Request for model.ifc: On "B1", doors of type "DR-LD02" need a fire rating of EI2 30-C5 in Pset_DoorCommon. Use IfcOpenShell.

First a look at what the model holds.

```python
import ifcopenshell
import ifcopenshell.util.element

model = ifcopenshell.open("model.ifc")
print(model.schema)
storey = next(s for s in model.by_type("IfcBuildingStorey") if s.Name == "B1")
doors = [e for e in ifcopenshell.util.element.get_decomposition(storey) if e.is_a("IfcDoor")]
seen = {}
for e in doors:
    element_type = ifcopenshell.util.element.get_type(e)
    key = (element_type.Name if element_type != e and element_type else None, ifcopenshell.util.element.get_pset(e, "Pset_DoorCommon", "FireRating"))
    seen[key] = seen.get(key, 0) + 1
for (name, value), count in sorted(seen.items(), key=str):
    print(count, "x", name, "|", value)
```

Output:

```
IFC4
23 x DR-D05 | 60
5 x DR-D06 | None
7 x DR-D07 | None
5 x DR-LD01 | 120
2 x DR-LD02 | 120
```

```python
import ifcopenshell
import ifcopenshell.api.pset
import ifcopenshell.util.element

model = ifcopenshell.open("model.ifc")

storey = next(s for s in model.by_type("IfcBuildingStorey") if s.Name == "B1")
doors = [e for e in ifcopenshell.util.element.get_decomposition(storey) if e.is_a("IfcDoor")]

count = 0
for e in doors:
    element_type = ifcopenshell.util.element.get_type(e)
    if element_type in (None, e) or element_type.Name != "DR-LD02":
        continue
    # add_pset returns the element's existing set when there is one.
    pset = ifcopenshell.api.pset.add_pset(model, product=e, name="Pset_DoorCommon")
    ifcopenshell.api.pset.edit_pset(model, pset=pset, properties={"FireRating": "EI2 30-C5"})
    count += 1

print(count, "doors updated")

model.write("model-out.ifc")
```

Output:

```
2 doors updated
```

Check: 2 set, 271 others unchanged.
